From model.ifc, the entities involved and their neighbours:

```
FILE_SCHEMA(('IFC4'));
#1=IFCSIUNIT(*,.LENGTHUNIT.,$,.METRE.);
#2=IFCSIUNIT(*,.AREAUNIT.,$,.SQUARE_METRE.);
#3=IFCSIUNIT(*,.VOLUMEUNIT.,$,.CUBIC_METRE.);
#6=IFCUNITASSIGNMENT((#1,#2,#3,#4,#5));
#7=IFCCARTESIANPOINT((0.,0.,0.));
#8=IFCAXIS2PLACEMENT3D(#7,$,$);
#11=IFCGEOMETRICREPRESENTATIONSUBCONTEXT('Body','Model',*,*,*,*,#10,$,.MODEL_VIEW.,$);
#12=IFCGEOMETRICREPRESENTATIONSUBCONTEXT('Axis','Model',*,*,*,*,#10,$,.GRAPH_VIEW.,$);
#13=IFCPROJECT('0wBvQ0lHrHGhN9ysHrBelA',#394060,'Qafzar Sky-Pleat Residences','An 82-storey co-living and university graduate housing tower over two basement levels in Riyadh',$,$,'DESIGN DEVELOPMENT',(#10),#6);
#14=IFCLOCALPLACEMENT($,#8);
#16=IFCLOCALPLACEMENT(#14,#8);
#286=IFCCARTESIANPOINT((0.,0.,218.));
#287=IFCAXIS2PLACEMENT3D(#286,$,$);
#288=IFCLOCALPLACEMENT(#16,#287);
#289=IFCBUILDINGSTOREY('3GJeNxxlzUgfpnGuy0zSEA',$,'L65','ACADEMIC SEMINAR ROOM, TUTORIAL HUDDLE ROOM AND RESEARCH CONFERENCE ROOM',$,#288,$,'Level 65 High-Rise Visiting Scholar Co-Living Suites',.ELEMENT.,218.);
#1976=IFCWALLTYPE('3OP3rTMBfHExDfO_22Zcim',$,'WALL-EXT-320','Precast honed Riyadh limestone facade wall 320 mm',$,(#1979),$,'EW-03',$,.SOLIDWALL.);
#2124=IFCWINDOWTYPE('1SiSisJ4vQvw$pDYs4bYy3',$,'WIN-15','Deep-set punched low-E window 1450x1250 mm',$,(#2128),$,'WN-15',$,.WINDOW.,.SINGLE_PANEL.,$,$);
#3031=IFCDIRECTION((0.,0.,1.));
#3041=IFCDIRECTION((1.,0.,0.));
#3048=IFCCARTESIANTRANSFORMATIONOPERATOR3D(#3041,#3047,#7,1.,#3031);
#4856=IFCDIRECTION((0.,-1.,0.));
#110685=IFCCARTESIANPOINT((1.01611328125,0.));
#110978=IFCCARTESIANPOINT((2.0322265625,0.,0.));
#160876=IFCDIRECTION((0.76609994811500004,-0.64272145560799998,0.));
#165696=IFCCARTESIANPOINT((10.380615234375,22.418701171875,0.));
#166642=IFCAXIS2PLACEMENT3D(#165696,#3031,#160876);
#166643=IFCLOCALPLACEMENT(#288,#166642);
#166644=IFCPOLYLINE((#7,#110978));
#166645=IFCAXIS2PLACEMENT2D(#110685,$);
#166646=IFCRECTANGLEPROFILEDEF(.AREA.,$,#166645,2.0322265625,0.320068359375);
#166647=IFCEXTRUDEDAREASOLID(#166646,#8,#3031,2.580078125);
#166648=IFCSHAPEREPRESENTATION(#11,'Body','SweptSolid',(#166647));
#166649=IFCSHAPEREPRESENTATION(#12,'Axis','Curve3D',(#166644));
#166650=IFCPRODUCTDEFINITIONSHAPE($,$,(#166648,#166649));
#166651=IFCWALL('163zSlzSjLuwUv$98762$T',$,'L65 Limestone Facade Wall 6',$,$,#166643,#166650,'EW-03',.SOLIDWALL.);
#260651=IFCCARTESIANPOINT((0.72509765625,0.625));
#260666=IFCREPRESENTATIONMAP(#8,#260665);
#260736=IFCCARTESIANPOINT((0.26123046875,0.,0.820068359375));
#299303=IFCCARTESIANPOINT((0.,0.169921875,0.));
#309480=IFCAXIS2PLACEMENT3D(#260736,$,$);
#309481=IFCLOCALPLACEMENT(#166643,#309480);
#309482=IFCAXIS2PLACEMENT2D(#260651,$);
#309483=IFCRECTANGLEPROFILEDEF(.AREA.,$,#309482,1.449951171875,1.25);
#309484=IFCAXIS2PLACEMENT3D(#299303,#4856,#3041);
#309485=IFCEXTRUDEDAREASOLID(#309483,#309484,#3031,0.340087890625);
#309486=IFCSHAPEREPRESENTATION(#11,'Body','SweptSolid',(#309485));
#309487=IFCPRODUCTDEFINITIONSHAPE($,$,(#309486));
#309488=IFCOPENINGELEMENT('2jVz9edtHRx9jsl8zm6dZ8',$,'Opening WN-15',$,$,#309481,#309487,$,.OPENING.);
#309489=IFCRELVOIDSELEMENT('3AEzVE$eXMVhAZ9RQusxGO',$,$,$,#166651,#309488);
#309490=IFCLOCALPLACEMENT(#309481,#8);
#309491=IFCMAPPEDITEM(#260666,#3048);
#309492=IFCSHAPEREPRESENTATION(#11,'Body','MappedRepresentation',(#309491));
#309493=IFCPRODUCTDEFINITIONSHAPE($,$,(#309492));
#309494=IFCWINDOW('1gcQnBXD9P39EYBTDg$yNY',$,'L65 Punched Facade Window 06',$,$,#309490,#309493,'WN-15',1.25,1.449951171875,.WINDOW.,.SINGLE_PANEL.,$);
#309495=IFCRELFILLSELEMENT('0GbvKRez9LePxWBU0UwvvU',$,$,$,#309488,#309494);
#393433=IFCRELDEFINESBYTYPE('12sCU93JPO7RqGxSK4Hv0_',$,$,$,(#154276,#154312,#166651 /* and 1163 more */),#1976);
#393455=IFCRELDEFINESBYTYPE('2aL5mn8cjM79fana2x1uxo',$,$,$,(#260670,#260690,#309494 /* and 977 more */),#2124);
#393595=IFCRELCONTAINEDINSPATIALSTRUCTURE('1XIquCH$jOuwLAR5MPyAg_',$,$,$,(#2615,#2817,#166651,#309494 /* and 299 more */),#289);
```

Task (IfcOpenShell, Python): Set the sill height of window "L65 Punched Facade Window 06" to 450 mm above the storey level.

```python
import numpy as np
import ifcopenshell
import ifcopenshell.api.geometry
import ifcopenshell.geom
import ifcopenshell.util.element
import ifcopenshell.util.placement
import ifcopenshell.util.shape
import ifcopenshell.util.unit

model = ifcopenshell.open("model.ifc")
unit_scale = ifcopenshell.util.unit.calculate_unit_scale(model)

window = model.by_id(309494)
opening = window.FillsVoids[0].RelatingOpeningElement
storey = ifcopenshell.util.element.get_container(window, ifc_class="IfcBuildingStorey")
level = ifcopenshell.util.placement.get_local_placement(storey.ObjectPlacement)[2, 3]

# The opening's origin need not be at the sill, so measure its lowest point.
shape = ifcopenshell.geom.create_shape(ifcopenshell.geom.settings(), opening)
bottom = ifcopenshell.util.shape.get_shape_bottom_elevation(shape, shape.geometry) / unit_scale
dz = level + 0.45 / unit_scale - bottom

shift = np.array([0.0, 0.0, dz])
# The window is placed relative to its opening, so it follows when the opening moves.
matrix = ifcopenshell.util.placement.get_local_placement(opening.ObjectPlacement)
matrix[:3, 3] += shift
ifcopenshell.api.geometry.edit_object_placement(
    model, product=opening, matrix=matrix, is_si=False, should_transform_children=True
)

print(f"moved by {dz * unit_scale:+.3f} m")

model.write("model_edited.ifc")
```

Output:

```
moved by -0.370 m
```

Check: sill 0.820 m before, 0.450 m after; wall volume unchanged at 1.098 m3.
